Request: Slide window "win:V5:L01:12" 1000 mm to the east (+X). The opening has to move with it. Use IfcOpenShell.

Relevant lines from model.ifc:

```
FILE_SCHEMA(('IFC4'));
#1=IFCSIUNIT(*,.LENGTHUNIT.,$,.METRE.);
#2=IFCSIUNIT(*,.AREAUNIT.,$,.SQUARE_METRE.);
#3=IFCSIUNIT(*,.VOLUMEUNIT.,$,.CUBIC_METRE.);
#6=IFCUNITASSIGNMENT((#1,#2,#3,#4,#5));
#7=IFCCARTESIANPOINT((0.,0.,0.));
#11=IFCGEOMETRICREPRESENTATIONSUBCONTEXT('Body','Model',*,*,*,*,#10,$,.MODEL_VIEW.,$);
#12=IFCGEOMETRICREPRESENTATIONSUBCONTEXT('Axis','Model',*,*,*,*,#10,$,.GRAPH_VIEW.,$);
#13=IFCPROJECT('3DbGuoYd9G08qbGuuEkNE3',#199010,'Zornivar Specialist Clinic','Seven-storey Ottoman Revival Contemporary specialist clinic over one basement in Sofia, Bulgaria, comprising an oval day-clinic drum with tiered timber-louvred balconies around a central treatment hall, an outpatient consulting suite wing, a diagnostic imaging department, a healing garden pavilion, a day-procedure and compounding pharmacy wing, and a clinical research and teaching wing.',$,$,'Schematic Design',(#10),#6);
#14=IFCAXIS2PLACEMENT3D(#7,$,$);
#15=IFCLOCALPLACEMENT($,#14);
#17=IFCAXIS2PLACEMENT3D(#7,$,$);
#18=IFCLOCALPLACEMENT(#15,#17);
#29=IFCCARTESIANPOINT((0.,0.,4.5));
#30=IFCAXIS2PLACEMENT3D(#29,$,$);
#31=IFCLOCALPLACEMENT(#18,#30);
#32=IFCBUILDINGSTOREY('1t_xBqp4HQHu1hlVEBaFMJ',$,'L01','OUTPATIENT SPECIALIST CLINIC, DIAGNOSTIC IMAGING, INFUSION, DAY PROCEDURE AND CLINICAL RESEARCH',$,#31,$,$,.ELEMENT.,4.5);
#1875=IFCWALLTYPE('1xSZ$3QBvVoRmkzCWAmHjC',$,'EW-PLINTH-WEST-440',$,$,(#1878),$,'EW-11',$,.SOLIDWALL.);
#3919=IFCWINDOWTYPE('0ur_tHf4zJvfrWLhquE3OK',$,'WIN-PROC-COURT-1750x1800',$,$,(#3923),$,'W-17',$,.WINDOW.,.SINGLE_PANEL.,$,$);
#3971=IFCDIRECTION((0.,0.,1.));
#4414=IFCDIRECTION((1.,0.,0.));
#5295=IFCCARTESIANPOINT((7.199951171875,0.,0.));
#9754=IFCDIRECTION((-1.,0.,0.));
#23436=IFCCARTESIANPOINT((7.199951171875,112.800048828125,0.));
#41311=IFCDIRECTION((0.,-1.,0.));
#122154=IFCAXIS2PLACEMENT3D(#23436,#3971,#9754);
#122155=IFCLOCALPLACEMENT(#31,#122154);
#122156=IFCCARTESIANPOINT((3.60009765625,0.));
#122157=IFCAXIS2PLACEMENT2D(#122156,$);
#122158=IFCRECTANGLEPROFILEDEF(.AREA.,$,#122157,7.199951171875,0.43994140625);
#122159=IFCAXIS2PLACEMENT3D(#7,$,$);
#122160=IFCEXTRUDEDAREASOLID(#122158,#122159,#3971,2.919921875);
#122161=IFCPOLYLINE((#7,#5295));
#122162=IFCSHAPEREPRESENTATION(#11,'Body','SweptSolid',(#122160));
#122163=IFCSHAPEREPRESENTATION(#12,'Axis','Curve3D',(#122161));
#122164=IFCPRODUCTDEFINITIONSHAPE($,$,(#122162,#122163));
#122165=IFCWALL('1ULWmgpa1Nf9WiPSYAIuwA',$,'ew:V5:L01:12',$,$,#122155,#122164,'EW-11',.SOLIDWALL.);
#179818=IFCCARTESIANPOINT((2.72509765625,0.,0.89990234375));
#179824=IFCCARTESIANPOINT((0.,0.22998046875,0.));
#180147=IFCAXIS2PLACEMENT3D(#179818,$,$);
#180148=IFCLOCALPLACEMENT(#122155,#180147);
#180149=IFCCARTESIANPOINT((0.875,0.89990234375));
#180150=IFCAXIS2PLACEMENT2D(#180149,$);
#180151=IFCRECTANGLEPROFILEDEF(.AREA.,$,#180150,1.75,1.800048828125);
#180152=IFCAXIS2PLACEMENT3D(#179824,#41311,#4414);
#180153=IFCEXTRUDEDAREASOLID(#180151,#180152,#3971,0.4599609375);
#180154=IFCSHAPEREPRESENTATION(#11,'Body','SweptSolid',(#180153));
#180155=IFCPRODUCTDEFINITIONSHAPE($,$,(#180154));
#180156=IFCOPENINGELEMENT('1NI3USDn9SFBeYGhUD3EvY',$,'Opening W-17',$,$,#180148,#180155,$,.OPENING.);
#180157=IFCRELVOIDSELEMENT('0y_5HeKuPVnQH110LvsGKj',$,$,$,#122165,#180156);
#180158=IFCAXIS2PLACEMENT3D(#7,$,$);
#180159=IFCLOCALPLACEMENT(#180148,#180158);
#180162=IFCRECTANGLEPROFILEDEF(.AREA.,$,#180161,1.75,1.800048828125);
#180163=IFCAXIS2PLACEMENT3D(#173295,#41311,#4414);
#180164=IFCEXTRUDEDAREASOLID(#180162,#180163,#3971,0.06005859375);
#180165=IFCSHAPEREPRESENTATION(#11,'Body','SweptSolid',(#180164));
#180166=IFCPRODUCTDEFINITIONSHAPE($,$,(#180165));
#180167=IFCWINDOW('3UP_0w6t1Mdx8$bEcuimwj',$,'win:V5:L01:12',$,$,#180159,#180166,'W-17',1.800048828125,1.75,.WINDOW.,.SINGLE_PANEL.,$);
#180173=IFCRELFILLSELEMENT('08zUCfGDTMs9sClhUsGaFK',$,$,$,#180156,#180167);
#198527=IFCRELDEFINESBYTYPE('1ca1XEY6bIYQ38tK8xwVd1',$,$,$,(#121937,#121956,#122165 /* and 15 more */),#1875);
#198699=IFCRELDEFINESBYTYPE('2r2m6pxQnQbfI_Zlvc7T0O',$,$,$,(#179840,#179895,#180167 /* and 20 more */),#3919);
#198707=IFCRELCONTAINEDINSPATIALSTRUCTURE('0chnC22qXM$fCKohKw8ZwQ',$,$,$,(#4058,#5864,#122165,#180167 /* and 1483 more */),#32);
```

```python
import ifcopenshell
import ifcopenshell.api.geometry
import ifcopenshell.util.placement

model = ifcopenshell.open("model.ifc")

window = model.by_guid("3UP_0w6t1Mdx8$bEcuimwj")
opening = window.FillsVoids[0].RelatingOpeningElement
wall = opening.VoidsElements[0].RelatingBuildingElement

wall_matrix = ifcopenshell.util.placement.get_local_placement(wall.ObjectPlacement)
shift = wall_matrix[:3, 0] * -1.0
before = ifcopenshell.util.placement.get_local_placement(window.ObjectPlacement)[:3, 3].copy()

# The window is placed relative to its opening, so it follows when the opening moves.
matrix = ifcopenshell.util.placement.get_local_placement(opening.ObjectPlacement)
matrix[:3, 3] += shift
ifcopenshell.api.geometry.edit_object_placement(
    model, product=opening, matrix=matrix, is_si=False, should_transform_children=True
)

after = ifcopenshell.util.placement.get_local_placement(window.ObjectPlacement)[:3, 3]
print("window moved by", (after - before).round(3) + 0.0)

model.write("model-out.ifc")
```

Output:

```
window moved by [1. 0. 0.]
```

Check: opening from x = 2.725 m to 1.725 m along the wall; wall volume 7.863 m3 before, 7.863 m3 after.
